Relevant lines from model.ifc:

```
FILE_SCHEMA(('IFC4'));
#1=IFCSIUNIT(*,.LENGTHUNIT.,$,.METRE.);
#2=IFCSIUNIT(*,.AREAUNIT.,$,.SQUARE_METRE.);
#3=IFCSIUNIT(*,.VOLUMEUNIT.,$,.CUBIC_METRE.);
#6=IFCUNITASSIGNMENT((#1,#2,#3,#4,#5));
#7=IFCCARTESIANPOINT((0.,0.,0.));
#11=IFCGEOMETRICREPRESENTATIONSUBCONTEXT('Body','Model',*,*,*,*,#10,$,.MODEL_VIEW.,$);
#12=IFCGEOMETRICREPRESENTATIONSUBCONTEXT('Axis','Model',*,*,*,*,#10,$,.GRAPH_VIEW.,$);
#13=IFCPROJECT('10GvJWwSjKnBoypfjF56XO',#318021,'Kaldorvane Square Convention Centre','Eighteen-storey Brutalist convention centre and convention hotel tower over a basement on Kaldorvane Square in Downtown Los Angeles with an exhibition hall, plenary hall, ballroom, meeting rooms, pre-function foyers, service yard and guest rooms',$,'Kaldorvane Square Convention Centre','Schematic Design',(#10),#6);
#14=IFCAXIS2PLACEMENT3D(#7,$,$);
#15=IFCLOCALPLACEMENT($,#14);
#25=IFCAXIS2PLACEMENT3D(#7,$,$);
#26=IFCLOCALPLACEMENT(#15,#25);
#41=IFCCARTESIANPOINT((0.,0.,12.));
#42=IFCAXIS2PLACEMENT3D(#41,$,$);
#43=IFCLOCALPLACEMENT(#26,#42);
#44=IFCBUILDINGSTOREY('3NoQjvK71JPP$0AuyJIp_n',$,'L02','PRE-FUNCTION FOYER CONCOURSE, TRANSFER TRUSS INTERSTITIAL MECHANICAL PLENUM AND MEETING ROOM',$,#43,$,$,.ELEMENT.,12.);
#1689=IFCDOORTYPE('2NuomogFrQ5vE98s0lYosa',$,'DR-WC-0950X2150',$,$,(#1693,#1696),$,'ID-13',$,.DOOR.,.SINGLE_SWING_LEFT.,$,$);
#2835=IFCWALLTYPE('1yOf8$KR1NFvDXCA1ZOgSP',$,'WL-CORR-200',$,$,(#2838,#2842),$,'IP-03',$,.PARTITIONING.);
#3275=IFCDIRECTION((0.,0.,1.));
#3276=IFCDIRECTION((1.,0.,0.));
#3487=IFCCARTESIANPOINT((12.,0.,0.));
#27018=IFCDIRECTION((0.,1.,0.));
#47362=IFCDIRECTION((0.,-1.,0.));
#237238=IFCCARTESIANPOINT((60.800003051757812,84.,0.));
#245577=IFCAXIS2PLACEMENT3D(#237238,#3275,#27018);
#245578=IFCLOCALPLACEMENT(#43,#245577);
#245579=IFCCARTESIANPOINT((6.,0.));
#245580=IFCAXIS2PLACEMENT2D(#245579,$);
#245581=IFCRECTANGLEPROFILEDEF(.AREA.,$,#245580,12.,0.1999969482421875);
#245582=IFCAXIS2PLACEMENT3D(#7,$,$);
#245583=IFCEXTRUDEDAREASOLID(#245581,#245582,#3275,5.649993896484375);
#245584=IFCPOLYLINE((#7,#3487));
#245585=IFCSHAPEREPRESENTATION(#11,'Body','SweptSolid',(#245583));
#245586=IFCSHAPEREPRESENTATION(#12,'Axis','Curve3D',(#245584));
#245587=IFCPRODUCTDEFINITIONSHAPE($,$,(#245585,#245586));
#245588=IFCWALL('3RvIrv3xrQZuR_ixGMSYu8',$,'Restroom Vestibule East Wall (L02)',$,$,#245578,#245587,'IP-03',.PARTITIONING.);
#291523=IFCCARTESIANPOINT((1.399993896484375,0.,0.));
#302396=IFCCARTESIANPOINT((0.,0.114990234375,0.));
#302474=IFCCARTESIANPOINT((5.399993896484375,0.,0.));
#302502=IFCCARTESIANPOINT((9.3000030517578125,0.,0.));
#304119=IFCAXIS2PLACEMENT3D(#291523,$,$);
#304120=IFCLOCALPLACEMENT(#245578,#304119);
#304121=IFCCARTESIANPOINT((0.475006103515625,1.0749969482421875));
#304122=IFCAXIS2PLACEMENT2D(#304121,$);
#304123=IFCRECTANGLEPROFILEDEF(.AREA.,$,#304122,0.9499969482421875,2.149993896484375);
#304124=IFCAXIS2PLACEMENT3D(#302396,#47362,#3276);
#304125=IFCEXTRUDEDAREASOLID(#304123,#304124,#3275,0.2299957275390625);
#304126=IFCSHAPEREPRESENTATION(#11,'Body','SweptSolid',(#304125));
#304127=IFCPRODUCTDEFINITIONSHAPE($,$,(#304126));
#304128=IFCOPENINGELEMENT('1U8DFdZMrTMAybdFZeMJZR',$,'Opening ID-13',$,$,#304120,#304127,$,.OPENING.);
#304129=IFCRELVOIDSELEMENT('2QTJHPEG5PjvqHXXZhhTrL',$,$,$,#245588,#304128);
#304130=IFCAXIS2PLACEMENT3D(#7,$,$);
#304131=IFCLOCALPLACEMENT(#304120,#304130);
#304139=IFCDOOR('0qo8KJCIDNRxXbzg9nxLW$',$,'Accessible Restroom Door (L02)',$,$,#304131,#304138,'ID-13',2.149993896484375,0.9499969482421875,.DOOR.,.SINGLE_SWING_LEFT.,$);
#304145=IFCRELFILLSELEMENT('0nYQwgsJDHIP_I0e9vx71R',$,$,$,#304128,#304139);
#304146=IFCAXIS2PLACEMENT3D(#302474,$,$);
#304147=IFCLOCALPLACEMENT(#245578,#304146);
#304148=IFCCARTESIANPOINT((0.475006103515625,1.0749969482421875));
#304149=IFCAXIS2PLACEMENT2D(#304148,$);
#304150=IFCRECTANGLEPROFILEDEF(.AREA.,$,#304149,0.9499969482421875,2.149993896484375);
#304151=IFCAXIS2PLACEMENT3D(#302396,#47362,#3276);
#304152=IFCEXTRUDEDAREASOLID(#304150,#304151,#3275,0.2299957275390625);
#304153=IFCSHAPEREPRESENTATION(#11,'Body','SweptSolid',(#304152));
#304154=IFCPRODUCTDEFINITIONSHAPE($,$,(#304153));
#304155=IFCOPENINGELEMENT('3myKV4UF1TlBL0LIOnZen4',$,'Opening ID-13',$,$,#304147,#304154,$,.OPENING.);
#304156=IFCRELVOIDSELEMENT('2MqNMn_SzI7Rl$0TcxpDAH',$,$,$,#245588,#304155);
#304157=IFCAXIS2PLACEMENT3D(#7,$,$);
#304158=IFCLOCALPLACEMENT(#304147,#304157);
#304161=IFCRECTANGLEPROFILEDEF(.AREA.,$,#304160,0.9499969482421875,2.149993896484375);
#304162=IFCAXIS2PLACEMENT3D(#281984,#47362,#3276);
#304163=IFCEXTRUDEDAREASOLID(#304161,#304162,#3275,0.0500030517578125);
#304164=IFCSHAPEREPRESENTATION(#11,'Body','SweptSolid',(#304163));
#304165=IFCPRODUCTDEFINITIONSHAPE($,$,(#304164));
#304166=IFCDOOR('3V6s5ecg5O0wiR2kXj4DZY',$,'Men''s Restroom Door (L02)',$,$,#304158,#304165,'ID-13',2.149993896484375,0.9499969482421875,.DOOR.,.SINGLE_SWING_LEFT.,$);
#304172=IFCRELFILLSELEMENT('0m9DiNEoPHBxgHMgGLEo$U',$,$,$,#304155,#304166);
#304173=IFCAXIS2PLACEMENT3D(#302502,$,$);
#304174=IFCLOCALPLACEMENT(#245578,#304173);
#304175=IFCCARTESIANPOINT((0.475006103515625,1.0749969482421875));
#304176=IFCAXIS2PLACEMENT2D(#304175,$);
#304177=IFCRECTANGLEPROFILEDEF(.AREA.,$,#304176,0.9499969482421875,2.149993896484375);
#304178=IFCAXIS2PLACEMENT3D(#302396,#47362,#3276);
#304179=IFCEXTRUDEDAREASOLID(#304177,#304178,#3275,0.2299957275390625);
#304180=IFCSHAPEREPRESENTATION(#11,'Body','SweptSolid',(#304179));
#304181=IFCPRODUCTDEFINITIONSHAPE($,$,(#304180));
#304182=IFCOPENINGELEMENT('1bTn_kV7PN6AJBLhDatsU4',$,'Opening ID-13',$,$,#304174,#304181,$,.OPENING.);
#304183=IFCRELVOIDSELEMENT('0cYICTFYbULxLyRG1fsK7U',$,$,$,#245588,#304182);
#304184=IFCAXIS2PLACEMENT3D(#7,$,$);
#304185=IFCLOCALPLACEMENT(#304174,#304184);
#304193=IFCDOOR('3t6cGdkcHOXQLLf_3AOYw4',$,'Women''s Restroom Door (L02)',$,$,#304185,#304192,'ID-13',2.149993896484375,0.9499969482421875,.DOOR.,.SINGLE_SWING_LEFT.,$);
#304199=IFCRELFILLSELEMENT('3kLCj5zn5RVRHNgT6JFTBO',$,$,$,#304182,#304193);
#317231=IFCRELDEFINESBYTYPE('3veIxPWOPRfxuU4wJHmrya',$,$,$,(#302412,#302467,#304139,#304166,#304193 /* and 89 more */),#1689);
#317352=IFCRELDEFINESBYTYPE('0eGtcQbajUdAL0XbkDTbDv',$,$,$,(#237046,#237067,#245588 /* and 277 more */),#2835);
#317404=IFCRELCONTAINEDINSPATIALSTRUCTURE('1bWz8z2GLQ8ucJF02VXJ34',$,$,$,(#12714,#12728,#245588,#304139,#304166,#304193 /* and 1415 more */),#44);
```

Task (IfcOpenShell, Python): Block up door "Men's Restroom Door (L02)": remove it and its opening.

```python
import ifcopenshell
import ifcopenshell.api.feature
import ifcopenshell.api.root
import ifcopenshell.geom
import ifcopenshell.util.shape

model = ifcopenshell.open("model.ifc")
settings = ifcopenshell.geom.settings()


def volume(element):
    """Net volume in cubic metres, openings subtracted."""
    shape = ifcopenshell.geom.create_shape(settings, element)
    return ifcopenshell.util.shape.get_volume(shape.geometry)


door = model.by_id(304166)
opening = door.FillsVoids[0].RelatingOpeningElement
wall = opening.VoidsElements[0].RelatingBuildingElement
before = volume(wall)

ifcopenshell.api.root.remove_product(model, product=door)
ifcopenshell.api.feature.remove_feature(model, feature=opening)

after = volume(wall)

print(f"wall volume {before:.3f} -> {after:.3f} m3")

model.write("model_updated.ifc")
```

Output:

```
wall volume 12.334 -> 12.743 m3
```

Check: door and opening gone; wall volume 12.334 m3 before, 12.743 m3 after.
